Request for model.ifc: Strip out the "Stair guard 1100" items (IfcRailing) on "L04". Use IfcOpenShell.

First a look at what the model holds.

```python
import ifcopenshell
import ifcopenshell.util.element

model = ifcopenshell.open("model.ifc")
print(model.schema)
storey = next(s for s in model.by_type("IfcBuildingStorey") if s.Name == "L04")
railings = [e for e in ifcopenshell.util.element.get_decomposition(storey) if e.is_a("IfcRailing")]
seen = {}
for e in railings:
    element_type = ifcopenshell.util.element.get_type(e)
    name = element_type.Name if element_type not in (None, e) else None
    seen[name] = seen.get(name, 0) + 1
for name, count in sorted(seen.items(), key=str):
    print(count, "x", name)
```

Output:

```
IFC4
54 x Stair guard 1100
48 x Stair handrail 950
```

```python
import ifcopenshell
import ifcopenshell.api.root
import ifcopenshell.util.element

model = ifcopenshell.open("model.ifc")

storey = next(s for s in model.by_type("IfcBuildingStorey") if s.Name == "L04")
railings = [e for e in ifcopenshell.util.element.get_decomposition(storey) if e.is_a("IfcRailing")]
targets = [e for e in railings if (t := ifcopenshell.util.element.get_type(e)) not in (None, e) and t.Name == "Stair guard 1100"]

for e in targets:
    ifcopenshell.api.root.remove_product(model, product=e)
print(len(targets), "removed")

model.write("model_v2.ifc")
```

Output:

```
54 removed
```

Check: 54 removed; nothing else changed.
